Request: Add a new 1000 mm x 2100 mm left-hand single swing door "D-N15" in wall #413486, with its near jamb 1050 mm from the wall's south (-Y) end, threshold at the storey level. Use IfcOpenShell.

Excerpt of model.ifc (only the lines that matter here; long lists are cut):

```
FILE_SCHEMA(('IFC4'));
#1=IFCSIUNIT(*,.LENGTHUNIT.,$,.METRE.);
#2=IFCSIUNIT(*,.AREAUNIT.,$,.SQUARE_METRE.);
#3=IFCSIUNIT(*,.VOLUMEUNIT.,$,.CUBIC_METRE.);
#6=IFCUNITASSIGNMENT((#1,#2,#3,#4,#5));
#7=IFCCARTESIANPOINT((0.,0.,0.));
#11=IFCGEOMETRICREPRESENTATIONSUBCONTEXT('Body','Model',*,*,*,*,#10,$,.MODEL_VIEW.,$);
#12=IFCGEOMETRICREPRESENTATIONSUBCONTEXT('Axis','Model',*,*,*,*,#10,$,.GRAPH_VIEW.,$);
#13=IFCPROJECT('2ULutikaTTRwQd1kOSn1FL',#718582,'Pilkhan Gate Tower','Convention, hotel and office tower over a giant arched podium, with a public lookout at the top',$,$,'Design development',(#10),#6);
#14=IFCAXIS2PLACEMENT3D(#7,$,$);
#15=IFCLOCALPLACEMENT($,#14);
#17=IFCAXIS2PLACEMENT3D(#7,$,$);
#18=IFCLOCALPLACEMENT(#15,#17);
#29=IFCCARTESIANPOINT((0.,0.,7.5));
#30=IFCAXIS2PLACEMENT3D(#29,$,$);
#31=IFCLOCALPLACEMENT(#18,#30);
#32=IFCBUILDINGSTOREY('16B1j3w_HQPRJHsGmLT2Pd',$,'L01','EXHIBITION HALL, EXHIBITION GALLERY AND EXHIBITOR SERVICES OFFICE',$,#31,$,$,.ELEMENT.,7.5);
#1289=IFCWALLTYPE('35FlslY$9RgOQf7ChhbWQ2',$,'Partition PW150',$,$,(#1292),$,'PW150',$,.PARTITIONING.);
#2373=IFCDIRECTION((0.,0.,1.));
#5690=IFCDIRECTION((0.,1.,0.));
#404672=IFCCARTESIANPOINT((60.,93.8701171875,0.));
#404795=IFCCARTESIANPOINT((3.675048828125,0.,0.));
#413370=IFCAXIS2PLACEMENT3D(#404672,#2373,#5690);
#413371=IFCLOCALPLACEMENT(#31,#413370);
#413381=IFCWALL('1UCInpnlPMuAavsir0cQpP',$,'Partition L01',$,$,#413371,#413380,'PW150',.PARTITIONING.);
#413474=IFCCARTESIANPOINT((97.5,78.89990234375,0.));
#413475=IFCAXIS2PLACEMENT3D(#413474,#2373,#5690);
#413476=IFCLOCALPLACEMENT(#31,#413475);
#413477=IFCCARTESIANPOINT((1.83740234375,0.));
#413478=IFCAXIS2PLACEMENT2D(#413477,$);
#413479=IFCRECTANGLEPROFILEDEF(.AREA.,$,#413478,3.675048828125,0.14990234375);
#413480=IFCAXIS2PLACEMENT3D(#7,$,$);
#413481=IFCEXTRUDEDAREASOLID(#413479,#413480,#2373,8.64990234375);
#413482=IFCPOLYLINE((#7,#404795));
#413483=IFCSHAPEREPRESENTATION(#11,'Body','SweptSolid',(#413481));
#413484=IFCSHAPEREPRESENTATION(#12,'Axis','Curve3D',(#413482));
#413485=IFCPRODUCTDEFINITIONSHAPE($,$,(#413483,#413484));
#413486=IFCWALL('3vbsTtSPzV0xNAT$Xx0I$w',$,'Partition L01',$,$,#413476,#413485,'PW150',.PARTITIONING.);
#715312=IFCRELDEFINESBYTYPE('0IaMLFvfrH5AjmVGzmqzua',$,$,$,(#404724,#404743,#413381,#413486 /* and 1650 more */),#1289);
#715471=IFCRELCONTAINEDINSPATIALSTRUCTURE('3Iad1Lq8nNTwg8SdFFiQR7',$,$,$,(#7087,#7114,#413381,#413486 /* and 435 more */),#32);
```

```python
import numpy as np
import ifcopenshell
import ifcopenshell.api.feature
import ifcopenshell.api.geometry
import ifcopenshell.api.root
import ifcopenshell.api.spatial
import ifcopenshell.geom
import ifcopenshell.util.element
import ifcopenshell.util.placement
import ifcopenshell.util.representation
import ifcopenshell.util.shape
import ifcopenshell.util.unit

model = ifcopenshell.open("model.ifc")
unit_scale = ifcopenshell.util.unit.calculate_unit_scale(model)
settings = ifcopenshell.geom.settings()


def volume(element):
    """Net volume in cubic metres, openings subtracted."""
    shape = ifcopenshell.geom.create_shape(settings, element)
    return ifcopenshell.util.shape.get_volume(shape.geometry)


wall = model.by_guid("3vbsTtSPzV0xNAT$Xx0I$w")
storey = ifcopenshell.util.element.get_container(wall, ifc_class="IfcBuildingStorey")
context = ifcopenshell.util.representation.get_context(model, "Model", "Body", "MODEL_VIEW")
before = volume(wall)

width, height, from_end, sill = 1, 2.1, 1.05, 0.0  # metres

# The wall runs along its own X axis, and the end named is its -X end.
wall_shape = ifcopenshell.geom.create_shape(settings, wall)
x, y, z = ifcopenshell.util.shape.get_vertices(wall_shape.geometry).T
start = x.min() + from_end
face, thickness = float(y.min()), float(y.max() - y.min())
wall_matrix = ifcopenshell.util.placement.get_local_placement(wall.ObjectPlacement)
level = ifcopenshell.util.placement.get_local_placement(storey.ObjectPlacement)[2, 3]


def in_wall(x, y):
    """Placement at x, y metres in the wall's axes, at sill height."""
    matrix = wall_matrix.copy()
    matrix[:, 3] = wall_matrix @ np.array([x / unit_scale, y / unit_scale, 0.0, 1.0])
    matrix[2, 3] = level + sill / unit_scale
    return matrix


# Opening: a box that overshoots both wall faces by 50 mm.
opening = ifcopenshell.api.root.create_entity(model, ifc_class="IfcOpeningElement", predefined_type="OPENING")
box = ifcopenshell.api.geometry.add_wall_representation(
    model, context=context, length=width, height=height, thickness=thickness + 0.1
)
ifcopenshell.api.geometry.assign_representation(model, product=opening, representation=box)
ifcopenshell.api.geometry.edit_object_placement(model, product=opening, matrix=in_wall(start, face - 0.05), is_si=False)
ifcopenshell.api.feature.add_feature(model, feature=opening, element=wall)

door = ifcopenshell.api.root.create_entity(model, ifc_class="IfcDoor", name="D-N15", predefined_type="DOOR")
door.OverallWidth, door.OverallHeight = width / unit_scale, height / unit_scale
door.OperationType = "SINGLE_SWING_LEFT"
body = ifcopenshell.api.geometry.add_door_representation(
    model,
    context=context,
    overall_width=door.OverallWidth,
    overall_height=door.OverallHeight,
    operation_type="SINGLE_SWING_LEFT",
    lining_properties={"LiningDepth": thickness / unit_scale, "ThresholdDepth": thickness / unit_scale},
)
ifcopenshell.api.geometry.assign_representation(model, product=door, representation=body)
ifcopenshell.api.spatial.assign_container(model, products=[door], relating_structure=storey)
ifcopenshell.api.feature.add_filling(model, opening=opening, element=door)

# The lining spans the wall, so the door starts at the wall face.
ifcopenshell.api.geometry.edit_object_placement(model, product=door, matrix=in_wall(start, face), is_si=False)

after = volume(wall)

print(f"wall volume {before:.3f} -> {after:.3f} m3")

model.write("model-out.ifc")
```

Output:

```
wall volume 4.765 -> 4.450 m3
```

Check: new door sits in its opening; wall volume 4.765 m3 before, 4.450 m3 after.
